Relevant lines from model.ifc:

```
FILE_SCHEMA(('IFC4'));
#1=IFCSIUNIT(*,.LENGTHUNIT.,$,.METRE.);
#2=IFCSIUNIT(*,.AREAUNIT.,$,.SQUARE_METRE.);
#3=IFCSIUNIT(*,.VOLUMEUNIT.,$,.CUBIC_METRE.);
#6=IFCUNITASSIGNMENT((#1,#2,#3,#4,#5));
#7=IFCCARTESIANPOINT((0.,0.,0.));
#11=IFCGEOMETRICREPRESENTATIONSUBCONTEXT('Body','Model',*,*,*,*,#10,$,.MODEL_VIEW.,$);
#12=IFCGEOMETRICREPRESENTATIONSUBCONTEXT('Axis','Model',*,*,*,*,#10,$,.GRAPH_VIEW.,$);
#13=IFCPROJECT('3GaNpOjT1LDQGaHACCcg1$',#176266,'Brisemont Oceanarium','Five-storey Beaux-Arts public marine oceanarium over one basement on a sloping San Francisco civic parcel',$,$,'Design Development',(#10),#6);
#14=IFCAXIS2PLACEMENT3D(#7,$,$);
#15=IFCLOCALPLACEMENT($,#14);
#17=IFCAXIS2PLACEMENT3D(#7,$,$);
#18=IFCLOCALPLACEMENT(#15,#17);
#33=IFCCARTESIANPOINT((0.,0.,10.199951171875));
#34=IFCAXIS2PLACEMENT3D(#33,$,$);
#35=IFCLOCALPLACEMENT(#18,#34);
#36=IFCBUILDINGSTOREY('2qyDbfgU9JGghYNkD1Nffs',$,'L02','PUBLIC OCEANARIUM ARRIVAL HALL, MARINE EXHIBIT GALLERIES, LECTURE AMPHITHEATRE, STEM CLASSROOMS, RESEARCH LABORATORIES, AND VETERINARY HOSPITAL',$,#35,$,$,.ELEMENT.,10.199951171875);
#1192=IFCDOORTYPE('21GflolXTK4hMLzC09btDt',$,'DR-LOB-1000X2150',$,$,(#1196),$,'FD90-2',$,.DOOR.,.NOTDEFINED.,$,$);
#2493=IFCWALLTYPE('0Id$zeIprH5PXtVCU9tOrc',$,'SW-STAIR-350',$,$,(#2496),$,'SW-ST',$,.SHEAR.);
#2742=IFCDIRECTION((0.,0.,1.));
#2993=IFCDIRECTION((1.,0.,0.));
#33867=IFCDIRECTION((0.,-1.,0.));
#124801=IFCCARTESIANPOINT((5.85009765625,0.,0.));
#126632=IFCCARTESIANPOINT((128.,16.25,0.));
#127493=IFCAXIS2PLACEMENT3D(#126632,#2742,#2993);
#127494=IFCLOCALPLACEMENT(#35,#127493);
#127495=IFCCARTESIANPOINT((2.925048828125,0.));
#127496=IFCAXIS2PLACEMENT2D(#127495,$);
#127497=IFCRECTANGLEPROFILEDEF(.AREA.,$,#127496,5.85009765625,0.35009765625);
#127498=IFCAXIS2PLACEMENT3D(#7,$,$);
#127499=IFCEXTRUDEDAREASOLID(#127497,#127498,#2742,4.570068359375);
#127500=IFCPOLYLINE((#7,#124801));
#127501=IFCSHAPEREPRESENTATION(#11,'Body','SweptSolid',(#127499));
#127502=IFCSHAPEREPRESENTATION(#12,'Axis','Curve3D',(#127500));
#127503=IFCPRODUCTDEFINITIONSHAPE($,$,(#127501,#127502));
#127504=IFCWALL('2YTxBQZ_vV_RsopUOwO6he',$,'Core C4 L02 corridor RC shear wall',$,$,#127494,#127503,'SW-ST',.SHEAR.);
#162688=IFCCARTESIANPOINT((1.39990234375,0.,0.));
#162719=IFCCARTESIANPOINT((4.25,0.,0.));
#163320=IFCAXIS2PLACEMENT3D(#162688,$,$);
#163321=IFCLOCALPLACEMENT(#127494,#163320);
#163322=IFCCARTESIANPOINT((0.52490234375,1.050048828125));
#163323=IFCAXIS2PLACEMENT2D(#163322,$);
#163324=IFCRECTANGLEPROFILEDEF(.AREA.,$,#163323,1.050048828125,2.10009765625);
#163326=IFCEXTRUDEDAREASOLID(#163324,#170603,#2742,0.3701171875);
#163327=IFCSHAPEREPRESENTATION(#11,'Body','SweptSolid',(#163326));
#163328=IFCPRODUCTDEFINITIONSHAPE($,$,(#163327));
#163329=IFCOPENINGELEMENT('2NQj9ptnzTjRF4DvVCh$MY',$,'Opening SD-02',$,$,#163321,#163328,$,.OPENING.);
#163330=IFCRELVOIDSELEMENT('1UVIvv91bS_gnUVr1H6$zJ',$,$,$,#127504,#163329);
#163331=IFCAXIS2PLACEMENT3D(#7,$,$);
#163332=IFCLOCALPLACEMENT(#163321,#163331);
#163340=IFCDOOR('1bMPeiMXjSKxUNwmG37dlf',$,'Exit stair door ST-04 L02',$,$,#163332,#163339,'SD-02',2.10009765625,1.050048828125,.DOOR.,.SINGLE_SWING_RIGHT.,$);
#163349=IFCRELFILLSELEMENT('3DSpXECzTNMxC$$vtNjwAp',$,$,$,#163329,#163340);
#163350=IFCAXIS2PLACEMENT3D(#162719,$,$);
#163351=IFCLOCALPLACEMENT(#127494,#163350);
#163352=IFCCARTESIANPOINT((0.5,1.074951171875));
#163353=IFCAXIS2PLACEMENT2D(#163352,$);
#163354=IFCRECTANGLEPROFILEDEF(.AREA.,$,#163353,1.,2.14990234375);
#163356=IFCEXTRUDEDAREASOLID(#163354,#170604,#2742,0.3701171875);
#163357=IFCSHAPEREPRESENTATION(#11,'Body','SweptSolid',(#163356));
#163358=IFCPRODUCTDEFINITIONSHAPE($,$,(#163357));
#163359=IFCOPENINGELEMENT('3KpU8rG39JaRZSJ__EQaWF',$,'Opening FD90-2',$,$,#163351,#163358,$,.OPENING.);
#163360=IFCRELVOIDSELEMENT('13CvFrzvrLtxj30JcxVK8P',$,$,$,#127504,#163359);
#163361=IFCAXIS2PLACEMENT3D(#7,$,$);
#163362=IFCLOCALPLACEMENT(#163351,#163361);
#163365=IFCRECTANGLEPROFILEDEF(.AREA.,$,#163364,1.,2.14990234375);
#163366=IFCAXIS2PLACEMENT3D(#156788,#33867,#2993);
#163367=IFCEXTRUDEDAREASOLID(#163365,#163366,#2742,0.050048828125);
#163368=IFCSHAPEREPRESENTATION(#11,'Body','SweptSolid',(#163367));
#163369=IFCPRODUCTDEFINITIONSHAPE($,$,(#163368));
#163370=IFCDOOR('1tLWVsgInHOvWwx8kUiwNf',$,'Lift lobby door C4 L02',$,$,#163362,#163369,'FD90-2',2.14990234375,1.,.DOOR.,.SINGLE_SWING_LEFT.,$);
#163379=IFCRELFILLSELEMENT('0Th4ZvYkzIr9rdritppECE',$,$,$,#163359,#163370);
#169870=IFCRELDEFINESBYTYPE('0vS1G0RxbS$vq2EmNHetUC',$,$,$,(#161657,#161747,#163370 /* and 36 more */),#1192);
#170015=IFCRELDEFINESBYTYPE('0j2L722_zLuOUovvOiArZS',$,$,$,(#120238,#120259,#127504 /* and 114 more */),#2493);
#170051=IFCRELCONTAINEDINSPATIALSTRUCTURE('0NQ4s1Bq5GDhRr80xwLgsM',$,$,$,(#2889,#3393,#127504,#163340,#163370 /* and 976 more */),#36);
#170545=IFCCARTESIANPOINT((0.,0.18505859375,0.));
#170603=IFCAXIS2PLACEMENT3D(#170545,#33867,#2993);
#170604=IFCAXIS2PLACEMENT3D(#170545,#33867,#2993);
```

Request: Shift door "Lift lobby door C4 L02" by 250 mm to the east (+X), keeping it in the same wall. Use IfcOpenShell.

```python
import ifcopenshell
import ifcopenshell.api.geometry
import ifcopenshell.util.placement

model = ifcopenshell.open("model.ifc")

door = model.by_id(163370)
opening = door.FillsVoids[0].RelatingOpeningElement
wall = opening.VoidsElements[0].RelatingBuildingElement

wall_matrix = ifcopenshell.util.placement.get_local_placement(wall.ObjectPlacement)
shift = wall_matrix[:3, 0] * 0.25
before = ifcopenshell.util.placement.get_local_placement(door.ObjectPlacement)[:3, 3].copy()

# The door is placed relative to its opening, so it follows when the opening moves.
matrix = ifcopenshell.util.placement.get_local_placement(opening.ObjectPlacement)
matrix[:3, 3] += shift
ifcopenshell.api.geometry.edit_object_placement(
    model, product=opening, matrix=matrix, is_si=False, should_transform_children=True
)

after = ifcopenshell.util.placement.get_local_placement(door.ObjectPlacement)[:3, 3]
print("door moved by", (after - before).round(3) + 0.0)

model.write("model_edited.ifc")
```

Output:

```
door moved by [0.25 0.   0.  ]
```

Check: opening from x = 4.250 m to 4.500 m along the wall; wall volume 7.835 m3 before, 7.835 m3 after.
